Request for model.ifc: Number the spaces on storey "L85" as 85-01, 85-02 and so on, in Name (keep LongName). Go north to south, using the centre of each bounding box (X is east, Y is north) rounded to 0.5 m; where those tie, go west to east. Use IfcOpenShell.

First a look at what the model holds.

```python
import ifcopenshell
import ifcopenshell.util.element
import ifcopenshell.util.placement

model = ifcopenshell.open("model.ifc")
print(model.schema)
storey = next(s for s in model.by_type("IfcBuildingStorey") if s.Name == "L85")
spaces = [e for e in ifcopenshell.util.element.get_decomposition(storey) if e.is_a("IfcSpace")]
for e in sorted(spaces, key=lambda e: e.id()):
    origin = ifcopenshell.util.placement.get_local_placement(e.ObjectPlacement)[:3, 3]
    print(e.id(), e.Name, e.LongName, origin.round(2) + 0.0, sep=" | ")
```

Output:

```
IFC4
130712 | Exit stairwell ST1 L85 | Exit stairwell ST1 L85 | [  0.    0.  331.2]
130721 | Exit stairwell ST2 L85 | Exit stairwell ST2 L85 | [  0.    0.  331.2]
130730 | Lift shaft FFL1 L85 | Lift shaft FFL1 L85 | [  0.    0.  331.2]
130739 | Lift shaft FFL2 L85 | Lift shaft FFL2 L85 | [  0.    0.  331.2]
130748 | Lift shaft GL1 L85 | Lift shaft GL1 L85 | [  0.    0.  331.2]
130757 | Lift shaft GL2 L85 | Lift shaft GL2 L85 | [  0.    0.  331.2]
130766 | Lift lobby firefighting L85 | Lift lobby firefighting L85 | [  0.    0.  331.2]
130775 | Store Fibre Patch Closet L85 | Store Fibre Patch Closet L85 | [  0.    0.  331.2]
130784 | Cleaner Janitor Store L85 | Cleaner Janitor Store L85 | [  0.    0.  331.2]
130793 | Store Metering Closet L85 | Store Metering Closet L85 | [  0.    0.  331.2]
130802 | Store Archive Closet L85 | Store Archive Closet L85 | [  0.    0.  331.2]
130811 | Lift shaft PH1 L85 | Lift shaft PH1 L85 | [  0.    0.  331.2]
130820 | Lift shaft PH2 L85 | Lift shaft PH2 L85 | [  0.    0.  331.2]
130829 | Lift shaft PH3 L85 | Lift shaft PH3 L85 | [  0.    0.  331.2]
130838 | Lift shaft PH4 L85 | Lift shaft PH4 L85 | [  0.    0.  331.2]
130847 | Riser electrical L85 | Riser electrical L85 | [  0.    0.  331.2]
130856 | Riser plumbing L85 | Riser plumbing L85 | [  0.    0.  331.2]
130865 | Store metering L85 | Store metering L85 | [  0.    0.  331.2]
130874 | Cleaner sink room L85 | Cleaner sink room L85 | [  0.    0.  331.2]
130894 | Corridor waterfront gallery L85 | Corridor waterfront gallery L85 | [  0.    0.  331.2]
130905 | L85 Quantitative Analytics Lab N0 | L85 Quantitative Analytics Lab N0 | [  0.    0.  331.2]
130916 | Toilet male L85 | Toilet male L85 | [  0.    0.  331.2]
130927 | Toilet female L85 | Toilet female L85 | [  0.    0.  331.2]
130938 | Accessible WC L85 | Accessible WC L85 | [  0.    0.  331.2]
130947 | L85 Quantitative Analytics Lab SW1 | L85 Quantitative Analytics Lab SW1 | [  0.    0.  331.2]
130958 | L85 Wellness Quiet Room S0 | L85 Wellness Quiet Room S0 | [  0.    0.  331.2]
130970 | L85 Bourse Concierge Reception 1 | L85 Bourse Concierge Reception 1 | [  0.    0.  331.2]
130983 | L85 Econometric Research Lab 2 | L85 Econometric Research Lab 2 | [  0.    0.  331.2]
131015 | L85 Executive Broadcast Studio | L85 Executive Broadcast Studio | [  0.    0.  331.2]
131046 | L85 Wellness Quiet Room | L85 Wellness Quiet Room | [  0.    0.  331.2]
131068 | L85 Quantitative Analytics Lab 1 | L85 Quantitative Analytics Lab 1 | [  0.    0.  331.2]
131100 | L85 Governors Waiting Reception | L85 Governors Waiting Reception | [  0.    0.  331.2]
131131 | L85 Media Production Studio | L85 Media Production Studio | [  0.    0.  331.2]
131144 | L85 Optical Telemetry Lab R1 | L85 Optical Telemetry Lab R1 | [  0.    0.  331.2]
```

```python
import ifcopenshell
import ifcopenshell.geom
import ifcopenshell.util.element
import ifcopenshell.util.shape

model = ifcopenshell.open("model.ifc")
settings = ifcopenshell.geom.settings()
settings.set("use-world-coords", True)


def centre(element):
    shape = ifcopenshell.geom.create_shape(settings, element)
    return ifcopenshell.util.shape.get_bbox_centroid(shape.geometry)


storey = next(s for s in model.by_type("IfcBuildingStorey") if s.Name == "L85")
spaces = [e for e in ifcopenshell.util.element.get_decomposition(storey) if e.is_a("IfcSpace")]

# Insertion points can sit at a corner or the storey origin, so sort by the geometry (in metres).
centres = {e: centre(e) for e in spaces}
spaces.sort(key=lambda e: (-round(centres[e][1] / 0.5), centres[e][0]))

for i, e in enumerate(spaces, start=1):
    number = f"85-{i:02d}"
    e.Name = number
    print(e.id(), number)

model.write("model_edited.ifc")
```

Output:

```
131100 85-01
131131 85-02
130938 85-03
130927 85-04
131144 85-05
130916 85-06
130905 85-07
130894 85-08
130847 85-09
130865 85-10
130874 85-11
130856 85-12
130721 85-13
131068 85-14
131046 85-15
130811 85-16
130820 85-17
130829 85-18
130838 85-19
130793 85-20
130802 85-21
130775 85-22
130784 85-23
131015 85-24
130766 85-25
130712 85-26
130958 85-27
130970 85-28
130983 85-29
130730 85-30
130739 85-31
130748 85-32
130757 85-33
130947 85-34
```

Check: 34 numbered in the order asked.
